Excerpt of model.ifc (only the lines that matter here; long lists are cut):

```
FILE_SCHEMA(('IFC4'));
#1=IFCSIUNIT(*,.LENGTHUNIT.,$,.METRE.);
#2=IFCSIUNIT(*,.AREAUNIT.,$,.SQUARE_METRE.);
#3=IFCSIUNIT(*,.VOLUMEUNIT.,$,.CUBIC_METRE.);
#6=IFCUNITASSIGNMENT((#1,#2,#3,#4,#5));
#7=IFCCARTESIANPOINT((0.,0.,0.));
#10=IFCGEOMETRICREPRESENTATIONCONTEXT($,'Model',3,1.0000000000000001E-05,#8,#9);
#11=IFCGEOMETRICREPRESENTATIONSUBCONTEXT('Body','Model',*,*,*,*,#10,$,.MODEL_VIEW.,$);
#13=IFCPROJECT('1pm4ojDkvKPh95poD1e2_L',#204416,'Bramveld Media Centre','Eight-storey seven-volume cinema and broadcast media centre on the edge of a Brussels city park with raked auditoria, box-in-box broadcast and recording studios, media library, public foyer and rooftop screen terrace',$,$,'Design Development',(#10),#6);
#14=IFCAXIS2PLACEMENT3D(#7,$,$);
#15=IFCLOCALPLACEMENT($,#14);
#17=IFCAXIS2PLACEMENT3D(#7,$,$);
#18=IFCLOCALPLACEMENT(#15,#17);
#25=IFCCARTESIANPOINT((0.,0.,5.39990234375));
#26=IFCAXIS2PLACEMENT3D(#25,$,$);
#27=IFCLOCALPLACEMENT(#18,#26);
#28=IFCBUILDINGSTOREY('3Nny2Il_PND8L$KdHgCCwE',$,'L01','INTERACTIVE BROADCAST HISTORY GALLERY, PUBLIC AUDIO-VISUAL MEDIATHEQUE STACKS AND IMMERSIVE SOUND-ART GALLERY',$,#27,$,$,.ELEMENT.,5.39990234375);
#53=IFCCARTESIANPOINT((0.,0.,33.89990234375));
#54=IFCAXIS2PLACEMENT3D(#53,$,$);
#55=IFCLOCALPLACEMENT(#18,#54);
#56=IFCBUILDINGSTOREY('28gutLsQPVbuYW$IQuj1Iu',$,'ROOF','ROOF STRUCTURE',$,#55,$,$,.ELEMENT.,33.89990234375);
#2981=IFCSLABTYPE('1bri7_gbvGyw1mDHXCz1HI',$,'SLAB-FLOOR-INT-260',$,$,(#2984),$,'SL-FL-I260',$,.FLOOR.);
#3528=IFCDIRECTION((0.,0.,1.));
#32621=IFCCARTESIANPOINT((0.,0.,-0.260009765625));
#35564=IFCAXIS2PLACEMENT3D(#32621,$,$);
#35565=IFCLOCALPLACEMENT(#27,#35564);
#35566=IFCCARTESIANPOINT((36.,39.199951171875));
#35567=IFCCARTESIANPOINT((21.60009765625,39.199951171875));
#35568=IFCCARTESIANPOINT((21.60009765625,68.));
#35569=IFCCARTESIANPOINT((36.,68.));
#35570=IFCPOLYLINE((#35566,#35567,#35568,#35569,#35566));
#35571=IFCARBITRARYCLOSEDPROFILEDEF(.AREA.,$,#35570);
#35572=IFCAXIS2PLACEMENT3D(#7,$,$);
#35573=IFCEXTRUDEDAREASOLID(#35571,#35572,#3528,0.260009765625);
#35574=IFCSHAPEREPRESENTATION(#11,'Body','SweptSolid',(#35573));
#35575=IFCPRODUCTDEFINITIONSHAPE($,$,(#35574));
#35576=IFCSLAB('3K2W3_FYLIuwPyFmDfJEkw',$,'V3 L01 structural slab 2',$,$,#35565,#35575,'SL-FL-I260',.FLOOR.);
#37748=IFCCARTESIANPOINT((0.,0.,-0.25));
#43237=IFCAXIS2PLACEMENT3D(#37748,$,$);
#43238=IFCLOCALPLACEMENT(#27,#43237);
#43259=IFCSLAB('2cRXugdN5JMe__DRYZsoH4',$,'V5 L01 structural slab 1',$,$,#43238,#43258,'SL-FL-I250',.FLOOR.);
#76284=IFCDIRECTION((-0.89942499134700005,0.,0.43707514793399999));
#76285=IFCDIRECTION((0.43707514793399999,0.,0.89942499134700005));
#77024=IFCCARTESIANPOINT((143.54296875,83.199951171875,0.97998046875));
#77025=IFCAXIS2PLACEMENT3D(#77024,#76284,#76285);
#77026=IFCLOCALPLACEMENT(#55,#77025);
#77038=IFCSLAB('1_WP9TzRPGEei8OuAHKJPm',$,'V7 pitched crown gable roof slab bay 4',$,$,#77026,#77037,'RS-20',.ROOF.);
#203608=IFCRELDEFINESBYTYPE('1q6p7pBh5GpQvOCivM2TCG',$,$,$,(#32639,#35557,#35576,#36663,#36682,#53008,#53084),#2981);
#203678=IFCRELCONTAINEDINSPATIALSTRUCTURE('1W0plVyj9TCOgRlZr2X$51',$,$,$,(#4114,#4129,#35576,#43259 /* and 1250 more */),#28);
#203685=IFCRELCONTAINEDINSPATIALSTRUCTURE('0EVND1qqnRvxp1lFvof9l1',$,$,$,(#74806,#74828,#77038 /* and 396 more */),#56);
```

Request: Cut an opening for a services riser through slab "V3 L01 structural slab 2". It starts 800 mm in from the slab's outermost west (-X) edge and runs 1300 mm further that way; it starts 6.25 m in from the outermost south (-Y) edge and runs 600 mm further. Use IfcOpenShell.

```python
import numpy as np
import ifcopenshell
import ifcopenshell.api.feature
import ifcopenshell.api.geometry
import ifcopenshell.api.root
import ifcopenshell.geom
import ifcopenshell.util.placement
import ifcopenshell.util.representation
import ifcopenshell.util.shape
import ifcopenshell.util.unit

model = ifcopenshell.open("model.ifc")
unit_scale = ifcopenshell.util.unit.calculate_unit_scale(model)
settings = ifcopenshell.geom.settings()


def volume(element):
    """Net volume in cubic metres, openings subtracted."""
    shape = ifcopenshell.geom.create_shape(settings, element)
    return ifcopenshell.util.shape.get_volume(shape.geometry)


slab = model.by_guid("3K2W3_FYLIuwPyFmDfJEkw")
before = volume(slab)

# Extent in the slab's own axes, in metres. The edges named are its -X and -Y sides.
slab_shape = ifcopenshell.geom.create_shape(settings, slab)
vertices = ifcopenshell.util.shape.get_vertices(slab_shape.geometry)
x_min, y_min, bottom = vertices.min(axis=0)
top = vertices[:, 2].max()

opening = ifcopenshell.api.root.create_entity(model, ifc_class="IfcOpeningElement", name="Services riser opening", predefined_type="OPENING")
context = ifcopenshell.util.representation.get_context(model, "Model", "Body", "MODEL_VIEW")
width, depth = 1.3, 0.6
outline = [(0.0, 0.0), (width, 0.0), (width, depth), (0.0, depth), (0.0, 0.0)]
# Overshoot both faces by 50 mm so the cut is clean.
shape = ifcopenshell.api.geometry.add_slab_representation(
    model, context=context, depth=top - bottom + 0.1, polyline=outline
)
ifcopenshell.api.geometry.assign_representation(model, product=opening, representation=shape)

matrix = ifcopenshell.util.placement.get_local_placement(slab.ObjectPlacement)
matrix[:, 3] = matrix @ np.append(np.array([x_min + 0.8, y_min + 6.25, bottom - 0.05]) / unit_scale, 1.0)
ifcopenshell.api.geometry.edit_object_placement(model, product=opening, matrix=matrix, is_si=False)
ifcopenshell.api.feature.add_feature(model, feature=opening, element=slab)

after = volume(slab)

print(f"slab volume {before:.3f} -> {after:.3f} m3")

model.write("model_edited.ifc")
```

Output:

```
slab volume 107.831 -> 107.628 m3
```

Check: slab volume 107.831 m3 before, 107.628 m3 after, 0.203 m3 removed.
